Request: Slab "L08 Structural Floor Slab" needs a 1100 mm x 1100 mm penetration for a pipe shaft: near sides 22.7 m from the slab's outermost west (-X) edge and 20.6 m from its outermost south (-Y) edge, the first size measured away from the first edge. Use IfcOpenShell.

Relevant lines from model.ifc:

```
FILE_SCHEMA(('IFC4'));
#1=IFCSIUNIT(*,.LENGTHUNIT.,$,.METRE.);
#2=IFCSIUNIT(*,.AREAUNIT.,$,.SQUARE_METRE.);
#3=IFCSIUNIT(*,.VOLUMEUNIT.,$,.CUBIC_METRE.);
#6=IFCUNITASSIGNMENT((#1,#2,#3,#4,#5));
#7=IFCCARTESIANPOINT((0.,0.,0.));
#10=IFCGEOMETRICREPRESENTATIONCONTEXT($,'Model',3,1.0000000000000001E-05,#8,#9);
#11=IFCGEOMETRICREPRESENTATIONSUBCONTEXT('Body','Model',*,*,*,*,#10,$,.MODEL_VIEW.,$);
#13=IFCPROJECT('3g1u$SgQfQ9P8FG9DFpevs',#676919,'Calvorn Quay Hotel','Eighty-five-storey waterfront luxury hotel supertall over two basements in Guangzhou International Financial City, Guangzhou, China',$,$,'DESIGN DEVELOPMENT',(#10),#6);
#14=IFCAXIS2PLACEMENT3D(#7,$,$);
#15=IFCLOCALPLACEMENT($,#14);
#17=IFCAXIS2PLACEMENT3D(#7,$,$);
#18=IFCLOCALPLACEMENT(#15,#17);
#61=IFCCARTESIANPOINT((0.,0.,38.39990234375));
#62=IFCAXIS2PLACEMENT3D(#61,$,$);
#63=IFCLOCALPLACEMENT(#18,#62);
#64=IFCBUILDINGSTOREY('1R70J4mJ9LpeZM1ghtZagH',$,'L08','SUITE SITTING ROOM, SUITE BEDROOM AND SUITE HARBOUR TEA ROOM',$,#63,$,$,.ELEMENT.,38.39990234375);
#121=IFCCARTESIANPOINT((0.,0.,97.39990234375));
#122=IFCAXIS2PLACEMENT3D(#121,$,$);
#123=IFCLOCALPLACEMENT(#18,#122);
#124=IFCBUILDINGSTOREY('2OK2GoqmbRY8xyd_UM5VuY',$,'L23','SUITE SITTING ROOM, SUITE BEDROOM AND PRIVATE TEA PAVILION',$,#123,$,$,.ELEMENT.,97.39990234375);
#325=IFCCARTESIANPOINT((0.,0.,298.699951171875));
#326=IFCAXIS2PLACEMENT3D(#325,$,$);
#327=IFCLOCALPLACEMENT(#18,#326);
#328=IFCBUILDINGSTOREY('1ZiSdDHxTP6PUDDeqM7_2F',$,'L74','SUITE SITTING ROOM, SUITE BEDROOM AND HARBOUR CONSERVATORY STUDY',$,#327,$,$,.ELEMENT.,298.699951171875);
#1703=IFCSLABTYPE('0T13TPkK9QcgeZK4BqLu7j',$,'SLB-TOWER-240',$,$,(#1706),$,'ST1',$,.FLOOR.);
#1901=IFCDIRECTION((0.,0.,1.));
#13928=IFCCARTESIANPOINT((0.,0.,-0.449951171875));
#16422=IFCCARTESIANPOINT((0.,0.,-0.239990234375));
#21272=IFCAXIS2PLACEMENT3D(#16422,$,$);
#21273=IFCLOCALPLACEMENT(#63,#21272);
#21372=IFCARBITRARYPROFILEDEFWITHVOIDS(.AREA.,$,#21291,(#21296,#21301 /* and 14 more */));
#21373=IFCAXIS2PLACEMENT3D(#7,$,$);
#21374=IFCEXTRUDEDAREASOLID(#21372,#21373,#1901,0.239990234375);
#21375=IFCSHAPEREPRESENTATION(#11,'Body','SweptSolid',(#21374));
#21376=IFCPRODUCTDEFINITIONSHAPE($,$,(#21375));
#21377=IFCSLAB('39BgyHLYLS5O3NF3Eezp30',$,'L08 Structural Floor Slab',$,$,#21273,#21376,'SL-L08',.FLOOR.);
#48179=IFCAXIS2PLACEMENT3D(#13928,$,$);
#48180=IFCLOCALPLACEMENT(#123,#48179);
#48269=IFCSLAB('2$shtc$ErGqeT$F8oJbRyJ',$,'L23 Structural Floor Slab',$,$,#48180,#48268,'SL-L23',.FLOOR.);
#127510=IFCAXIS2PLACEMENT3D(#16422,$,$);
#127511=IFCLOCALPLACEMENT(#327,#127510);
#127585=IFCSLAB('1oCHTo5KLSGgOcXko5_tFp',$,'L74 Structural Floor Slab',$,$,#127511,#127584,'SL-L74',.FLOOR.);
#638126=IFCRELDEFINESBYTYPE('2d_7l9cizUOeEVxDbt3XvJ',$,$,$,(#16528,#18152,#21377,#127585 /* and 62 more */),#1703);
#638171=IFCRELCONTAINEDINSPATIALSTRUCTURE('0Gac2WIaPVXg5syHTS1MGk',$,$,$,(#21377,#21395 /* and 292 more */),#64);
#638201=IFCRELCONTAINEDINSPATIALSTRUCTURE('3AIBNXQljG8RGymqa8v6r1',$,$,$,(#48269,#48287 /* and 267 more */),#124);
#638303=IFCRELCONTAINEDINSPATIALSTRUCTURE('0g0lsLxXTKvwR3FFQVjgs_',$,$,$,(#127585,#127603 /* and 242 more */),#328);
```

```python
import numpy as np
import ifcopenshell
import ifcopenshell.api.feature
import ifcopenshell.api.geometry
import ifcopenshell.api.root
import ifcopenshell.geom
import ifcopenshell.util.placement
import ifcopenshell.util.representation
import ifcopenshell.util.shape
import ifcopenshell.util.unit

model = ifcopenshell.open("model.ifc")
unit_scale = ifcopenshell.util.unit.calculate_unit_scale(model)
settings = ifcopenshell.geom.settings()


def volume(element):
    """Net volume in cubic metres, openings subtracted."""
    shape = ifcopenshell.geom.create_shape(settings, element)
    return ifcopenshell.util.shape.get_volume(shape.geometry)


slab = model.by_guid("39BgyHLYLS5O3NF3Eezp30")
before = volume(slab)

# Extent in the slab's own axes, in metres. The edges named are its -X and -Y sides.
slab_shape = ifcopenshell.geom.create_shape(settings, slab)
vertices = ifcopenshell.util.shape.get_vertices(slab_shape.geometry)
x_min, y_min, bottom = vertices.min(axis=0)
top = vertices[:, 2].max()

opening = ifcopenshell.api.root.create_entity(model, ifc_class="IfcOpeningElement", name="Pipe shaft opening", predefined_type="OPENING")
context = ifcopenshell.util.representation.get_context(model, "Model", "Body", "MODEL_VIEW")
width, depth = 1.1, 1.1
outline = [(0.0, 0.0), (width, 0.0), (width, depth), (0.0, depth), (0.0, 0.0)]
# Overshoot both faces by 50 mm so the cut is clean.
shape = ifcopenshell.api.geometry.add_slab_representation(
    model, context=context, depth=top - bottom + 0.1, polyline=outline
)
ifcopenshell.api.geometry.assign_representation(model, product=opening, representation=shape)

matrix = ifcopenshell.util.placement.get_local_placement(slab.ObjectPlacement)
matrix[:, 3] = matrix @ np.append(np.array([x_min + 22.7, y_min + 20.6, bottom - 0.05]) / unit_scale, 1.0)
ifcopenshell.api.geometry.edit_object_placement(model, product=opening, matrix=matrix, is_si=False)
ifcopenshell.api.feature.add_feature(model, feature=opening, element=slab)

after = volume(slab)

print(f"slab volume {before:.3f} -> {after:.3f} m3")

model.write("model-out.ifc")
```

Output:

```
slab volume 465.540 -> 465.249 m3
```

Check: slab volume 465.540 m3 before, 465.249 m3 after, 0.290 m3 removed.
